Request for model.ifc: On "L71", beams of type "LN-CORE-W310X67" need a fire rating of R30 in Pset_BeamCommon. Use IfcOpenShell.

First a look at what the model holds.

```python
import ifcopenshell
import ifcopenshell.util.element

model = ifcopenshell.open("model.ifc")
print(model.schema)
storey = next(s for s in model.by_type("IfcBuildingStorey") if s.Name == "L71")
beams = [e for e in ifcopenshell.util.element.get_decomposition(storey) if e.is_a("IfcBeam")]
seen = {}
for e in beams:
    element_type = ifcopenshell.util.element.get_type(e)
    key = (element_type.Name if element_type != e and element_type else None, ifcopenshell.util.element.get_pset(e, "Pset_BeamCommon", "FireRating"))
    seen[key] = seen.get(key, 0) + 1
for (name, value), count in sorted(seen.items(), key=str):
    print(count, "x", name, "|", value)
```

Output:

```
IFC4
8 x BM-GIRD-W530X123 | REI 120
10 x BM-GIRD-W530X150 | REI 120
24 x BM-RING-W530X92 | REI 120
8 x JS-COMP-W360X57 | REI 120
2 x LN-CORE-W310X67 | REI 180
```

```python
import ifcopenshell
import ifcopenshell.api.pset
import ifcopenshell.util.element

model = ifcopenshell.open("model.ifc")

storey = next(s for s in model.by_type("IfcBuildingStorey") if s.Name == "L71")
beams = [e for e in ifcopenshell.util.element.get_decomposition(storey) if e.is_a("IfcBeam")]

count = 0
for e in beams:
    element_type = ifcopenshell.util.element.get_type(e)
    if element_type in (None, e) or element_type.Name != "LN-CORE-W310X67":
        continue
    found = ifcopenshell.util.element.get_pset(e, "Pset_BeamCommon", should_inherit=False)
    if found:
        pset = model.by_id(found["id"])
        if len(ifcopenshell.util.element.get_elements_by_pset(pset)) > 1:
            pset = ifcopenshell.api.pset.unshare_pset(model, products=[e], pset=pset)[0]
    else:
        pset = ifcopenshell.api.pset.add_pset(model, product=e, name="Pset_BeamCommon")
    ifcopenshell.api.pset.edit_pset(model, pset=pset, properties={"FireRating": "R30"})
    count += 1

print(count, "beams updated")

model.write("model_updated.ifc")
```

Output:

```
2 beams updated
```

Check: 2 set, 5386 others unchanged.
